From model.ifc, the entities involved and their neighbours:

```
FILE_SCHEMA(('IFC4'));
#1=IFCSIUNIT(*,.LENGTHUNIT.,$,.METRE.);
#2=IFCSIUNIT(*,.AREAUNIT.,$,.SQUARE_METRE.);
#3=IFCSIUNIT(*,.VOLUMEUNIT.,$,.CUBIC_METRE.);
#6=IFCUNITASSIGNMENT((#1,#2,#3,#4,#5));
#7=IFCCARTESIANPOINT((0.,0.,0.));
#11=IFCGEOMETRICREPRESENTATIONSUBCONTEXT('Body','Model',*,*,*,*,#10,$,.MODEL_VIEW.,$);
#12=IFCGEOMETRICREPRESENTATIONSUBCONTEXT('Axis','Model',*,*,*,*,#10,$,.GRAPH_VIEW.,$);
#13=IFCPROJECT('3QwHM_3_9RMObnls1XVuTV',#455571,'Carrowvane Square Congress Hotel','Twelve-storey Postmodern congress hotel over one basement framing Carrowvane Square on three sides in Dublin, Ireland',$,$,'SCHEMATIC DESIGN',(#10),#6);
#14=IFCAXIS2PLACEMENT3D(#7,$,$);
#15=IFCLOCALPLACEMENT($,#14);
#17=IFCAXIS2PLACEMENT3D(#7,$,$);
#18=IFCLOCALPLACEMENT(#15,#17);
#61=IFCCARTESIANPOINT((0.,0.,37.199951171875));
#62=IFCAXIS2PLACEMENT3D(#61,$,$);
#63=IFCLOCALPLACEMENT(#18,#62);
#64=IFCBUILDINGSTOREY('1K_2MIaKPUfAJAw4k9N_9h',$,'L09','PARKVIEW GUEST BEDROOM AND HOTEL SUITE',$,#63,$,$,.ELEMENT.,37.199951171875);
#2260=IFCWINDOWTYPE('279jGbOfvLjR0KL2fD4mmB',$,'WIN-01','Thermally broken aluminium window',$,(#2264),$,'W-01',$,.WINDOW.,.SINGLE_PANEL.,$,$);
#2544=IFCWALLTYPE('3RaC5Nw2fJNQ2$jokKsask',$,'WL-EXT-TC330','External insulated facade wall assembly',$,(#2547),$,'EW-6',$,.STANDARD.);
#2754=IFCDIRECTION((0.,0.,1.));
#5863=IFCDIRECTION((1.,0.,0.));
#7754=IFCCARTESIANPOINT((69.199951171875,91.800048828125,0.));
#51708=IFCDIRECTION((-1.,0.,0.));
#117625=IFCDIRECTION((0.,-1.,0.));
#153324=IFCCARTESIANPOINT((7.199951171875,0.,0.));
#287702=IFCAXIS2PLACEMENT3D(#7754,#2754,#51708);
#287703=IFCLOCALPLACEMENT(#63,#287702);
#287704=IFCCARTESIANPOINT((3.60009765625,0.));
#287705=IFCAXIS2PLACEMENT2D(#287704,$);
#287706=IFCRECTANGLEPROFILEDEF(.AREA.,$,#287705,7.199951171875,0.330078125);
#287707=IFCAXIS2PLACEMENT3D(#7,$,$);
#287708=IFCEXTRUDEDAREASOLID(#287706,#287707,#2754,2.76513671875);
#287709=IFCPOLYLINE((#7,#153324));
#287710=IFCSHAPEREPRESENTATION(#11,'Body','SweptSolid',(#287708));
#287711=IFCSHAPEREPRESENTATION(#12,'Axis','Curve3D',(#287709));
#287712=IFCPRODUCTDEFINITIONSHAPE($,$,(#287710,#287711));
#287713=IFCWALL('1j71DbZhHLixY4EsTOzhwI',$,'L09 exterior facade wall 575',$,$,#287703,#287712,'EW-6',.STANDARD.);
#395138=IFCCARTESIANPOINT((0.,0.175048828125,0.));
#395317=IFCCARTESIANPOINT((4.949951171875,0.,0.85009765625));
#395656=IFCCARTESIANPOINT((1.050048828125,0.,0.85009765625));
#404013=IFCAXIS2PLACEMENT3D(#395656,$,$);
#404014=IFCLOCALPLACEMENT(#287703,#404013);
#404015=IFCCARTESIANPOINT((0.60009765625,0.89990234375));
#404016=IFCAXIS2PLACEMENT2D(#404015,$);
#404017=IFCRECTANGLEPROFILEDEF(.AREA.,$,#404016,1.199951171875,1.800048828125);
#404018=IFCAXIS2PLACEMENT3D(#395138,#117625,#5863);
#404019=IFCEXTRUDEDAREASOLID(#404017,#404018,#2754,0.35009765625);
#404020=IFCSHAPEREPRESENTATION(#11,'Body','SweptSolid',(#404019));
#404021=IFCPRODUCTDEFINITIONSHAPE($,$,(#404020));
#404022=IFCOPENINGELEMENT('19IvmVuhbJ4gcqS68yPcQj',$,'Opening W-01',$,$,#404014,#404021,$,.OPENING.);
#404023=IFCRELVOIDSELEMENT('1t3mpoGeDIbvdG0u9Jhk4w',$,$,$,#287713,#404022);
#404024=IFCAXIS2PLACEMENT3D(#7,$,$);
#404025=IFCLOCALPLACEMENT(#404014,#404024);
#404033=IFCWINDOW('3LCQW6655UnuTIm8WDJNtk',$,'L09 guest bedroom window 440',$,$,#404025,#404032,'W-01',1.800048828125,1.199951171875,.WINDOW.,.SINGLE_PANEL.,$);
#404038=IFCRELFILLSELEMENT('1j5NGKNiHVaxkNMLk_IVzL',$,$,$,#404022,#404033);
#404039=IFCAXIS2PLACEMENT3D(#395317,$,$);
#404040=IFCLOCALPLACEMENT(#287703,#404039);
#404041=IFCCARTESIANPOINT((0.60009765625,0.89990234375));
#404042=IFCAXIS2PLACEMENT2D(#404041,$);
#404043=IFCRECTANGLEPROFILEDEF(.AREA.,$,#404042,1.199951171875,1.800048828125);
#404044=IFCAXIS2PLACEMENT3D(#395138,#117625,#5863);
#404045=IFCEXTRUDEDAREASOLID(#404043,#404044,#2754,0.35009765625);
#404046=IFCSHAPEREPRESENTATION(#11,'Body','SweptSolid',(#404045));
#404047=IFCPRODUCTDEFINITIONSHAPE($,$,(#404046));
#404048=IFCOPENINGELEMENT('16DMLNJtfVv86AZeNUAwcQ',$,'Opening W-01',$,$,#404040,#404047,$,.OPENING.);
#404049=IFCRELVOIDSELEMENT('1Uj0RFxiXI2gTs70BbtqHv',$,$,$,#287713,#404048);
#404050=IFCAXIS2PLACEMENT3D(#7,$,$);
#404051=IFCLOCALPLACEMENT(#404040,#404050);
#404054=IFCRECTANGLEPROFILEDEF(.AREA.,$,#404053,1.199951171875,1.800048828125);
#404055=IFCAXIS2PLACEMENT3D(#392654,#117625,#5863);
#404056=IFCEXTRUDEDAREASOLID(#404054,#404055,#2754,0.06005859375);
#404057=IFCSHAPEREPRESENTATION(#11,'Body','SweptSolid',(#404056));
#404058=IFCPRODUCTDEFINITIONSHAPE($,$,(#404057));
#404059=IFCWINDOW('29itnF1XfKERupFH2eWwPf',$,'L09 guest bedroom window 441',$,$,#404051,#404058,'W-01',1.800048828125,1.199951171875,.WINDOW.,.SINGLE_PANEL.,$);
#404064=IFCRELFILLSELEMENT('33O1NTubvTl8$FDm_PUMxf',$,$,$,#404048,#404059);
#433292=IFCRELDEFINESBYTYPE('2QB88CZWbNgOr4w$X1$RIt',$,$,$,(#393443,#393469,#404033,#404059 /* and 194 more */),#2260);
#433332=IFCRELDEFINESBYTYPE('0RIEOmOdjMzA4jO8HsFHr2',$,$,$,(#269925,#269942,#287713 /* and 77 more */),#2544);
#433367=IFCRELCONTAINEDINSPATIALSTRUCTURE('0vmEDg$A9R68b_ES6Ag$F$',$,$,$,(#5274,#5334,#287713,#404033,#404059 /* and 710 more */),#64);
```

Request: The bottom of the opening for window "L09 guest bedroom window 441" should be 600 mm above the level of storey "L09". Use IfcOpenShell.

```python
import numpy as np
import ifcopenshell
import ifcopenshell.api.geometry
import ifcopenshell.geom
import ifcopenshell.util.element
import ifcopenshell.util.placement
import ifcopenshell.util.shape
import ifcopenshell.util.unit

model = ifcopenshell.open("model.ifc")
unit_scale = ifcopenshell.util.unit.calculate_unit_scale(model)

window = model.by_guid("29itnF1XfKERupFH2eWwPf")
opening = window.FillsVoids[0].RelatingOpeningElement
storey = ifcopenshell.util.element.get_container(window, ifc_class="IfcBuildingStorey")
level = ifcopenshell.util.placement.get_local_placement(storey.ObjectPlacement)[2, 3]

# The opening's origin need not be at the sill, so measure its lowest point.
shape = ifcopenshell.geom.create_shape(ifcopenshell.geom.settings(), opening)
bottom = ifcopenshell.util.shape.get_shape_bottom_elevation(shape, shape.geometry) / unit_scale
dz = level + 0.6 - bottom

shift = np.array([0.0, 0.0, dz])
# The window is placed relative to its opening, so it follows when the opening moves.
matrix = ifcopenshell.util.placement.get_local_placement(opening.ObjectPlacement)
matrix[:3, 3] += shift
ifcopenshell.api.geometry.edit_object_placement(
    model, product=opening, matrix=matrix, is_si=False, should_transform_children=True
)

print(f"moved by {dz * unit_scale:+.3f} m")

model.write("model_edited.ifc")
```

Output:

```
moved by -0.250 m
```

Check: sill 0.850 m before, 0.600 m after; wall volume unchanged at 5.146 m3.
